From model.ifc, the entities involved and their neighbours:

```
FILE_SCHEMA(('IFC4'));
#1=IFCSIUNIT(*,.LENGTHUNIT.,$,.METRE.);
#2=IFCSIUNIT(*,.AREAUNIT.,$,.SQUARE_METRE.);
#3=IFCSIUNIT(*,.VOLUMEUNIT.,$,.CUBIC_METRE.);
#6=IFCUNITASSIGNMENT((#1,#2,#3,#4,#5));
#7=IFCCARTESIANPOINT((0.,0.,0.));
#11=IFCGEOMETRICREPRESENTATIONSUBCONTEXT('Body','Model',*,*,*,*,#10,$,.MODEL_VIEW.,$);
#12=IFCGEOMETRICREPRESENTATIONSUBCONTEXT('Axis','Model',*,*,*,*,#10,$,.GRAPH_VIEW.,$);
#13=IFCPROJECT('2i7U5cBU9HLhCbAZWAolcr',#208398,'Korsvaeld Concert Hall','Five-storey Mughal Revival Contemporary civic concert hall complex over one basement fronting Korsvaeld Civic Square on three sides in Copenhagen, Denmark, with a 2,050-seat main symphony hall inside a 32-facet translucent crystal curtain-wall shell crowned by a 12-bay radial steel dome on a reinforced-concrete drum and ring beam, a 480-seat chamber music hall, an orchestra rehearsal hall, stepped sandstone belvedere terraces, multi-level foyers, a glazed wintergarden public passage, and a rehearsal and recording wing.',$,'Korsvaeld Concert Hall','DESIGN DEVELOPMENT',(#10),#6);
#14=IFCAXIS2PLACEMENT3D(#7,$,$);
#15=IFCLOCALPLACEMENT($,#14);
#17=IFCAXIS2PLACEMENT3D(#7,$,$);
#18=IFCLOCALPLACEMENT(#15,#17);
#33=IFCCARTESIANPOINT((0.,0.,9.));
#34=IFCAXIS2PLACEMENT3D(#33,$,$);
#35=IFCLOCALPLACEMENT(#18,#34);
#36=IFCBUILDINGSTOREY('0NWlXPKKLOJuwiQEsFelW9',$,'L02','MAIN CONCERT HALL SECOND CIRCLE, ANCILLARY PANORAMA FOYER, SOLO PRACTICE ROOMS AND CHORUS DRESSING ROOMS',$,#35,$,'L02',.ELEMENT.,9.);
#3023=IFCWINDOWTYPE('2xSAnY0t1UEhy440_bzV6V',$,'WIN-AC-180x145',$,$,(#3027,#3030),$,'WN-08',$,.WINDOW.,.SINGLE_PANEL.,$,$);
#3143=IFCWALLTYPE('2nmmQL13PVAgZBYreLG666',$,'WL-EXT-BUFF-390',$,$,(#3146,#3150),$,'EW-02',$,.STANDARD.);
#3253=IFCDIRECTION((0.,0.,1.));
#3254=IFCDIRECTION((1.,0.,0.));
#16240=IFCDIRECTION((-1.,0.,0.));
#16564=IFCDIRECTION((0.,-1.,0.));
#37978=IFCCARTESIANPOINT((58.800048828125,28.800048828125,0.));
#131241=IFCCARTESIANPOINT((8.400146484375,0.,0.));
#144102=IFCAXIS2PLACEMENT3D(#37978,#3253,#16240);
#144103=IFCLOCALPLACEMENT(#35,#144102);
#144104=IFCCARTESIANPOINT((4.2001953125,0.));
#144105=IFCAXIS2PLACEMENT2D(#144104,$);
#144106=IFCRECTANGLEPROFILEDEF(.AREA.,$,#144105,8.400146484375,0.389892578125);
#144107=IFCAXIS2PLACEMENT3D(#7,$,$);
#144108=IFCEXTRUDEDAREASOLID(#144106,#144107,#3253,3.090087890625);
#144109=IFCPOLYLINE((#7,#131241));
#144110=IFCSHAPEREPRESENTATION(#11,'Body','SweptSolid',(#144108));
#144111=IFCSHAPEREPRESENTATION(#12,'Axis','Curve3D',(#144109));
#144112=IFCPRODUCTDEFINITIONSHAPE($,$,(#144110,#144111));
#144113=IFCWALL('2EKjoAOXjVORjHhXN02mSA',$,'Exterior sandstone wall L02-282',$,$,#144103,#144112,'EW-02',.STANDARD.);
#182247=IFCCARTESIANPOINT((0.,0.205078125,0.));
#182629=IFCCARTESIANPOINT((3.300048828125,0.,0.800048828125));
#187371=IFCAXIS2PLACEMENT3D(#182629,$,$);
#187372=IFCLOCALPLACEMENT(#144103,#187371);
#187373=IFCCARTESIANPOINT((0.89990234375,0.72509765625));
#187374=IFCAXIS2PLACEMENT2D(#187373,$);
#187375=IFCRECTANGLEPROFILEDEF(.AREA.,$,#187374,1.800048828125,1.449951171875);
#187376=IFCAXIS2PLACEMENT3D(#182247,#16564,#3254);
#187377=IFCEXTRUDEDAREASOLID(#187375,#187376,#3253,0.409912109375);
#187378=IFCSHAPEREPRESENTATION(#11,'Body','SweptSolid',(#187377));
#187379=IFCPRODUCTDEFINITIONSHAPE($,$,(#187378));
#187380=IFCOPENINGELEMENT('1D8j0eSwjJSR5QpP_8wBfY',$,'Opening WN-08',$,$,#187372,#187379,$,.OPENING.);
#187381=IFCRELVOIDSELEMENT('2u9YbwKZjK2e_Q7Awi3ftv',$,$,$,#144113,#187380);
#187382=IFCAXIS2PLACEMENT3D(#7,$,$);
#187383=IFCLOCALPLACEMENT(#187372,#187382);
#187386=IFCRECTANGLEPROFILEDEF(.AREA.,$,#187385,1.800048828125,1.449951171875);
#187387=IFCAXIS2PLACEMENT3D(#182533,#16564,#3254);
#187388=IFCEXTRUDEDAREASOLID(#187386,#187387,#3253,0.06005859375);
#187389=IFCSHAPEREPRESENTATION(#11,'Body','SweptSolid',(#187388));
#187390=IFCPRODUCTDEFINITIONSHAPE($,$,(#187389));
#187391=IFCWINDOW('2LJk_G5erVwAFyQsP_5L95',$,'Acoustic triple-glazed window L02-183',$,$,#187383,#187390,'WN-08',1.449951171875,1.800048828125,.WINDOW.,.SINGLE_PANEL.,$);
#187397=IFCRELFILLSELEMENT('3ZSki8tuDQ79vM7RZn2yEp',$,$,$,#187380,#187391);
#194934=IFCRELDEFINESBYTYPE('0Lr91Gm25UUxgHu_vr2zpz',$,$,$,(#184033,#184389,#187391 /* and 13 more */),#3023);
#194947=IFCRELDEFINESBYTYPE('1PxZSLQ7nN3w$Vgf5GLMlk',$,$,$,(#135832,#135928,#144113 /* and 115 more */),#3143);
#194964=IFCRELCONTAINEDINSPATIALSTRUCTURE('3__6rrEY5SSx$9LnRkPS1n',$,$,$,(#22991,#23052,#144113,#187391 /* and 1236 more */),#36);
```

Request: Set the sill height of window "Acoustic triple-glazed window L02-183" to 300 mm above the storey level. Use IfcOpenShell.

```python
import numpy as np
import ifcopenshell
import ifcopenshell.api.geometry
import ifcopenshell.geom
import ifcopenshell.util.element
import ifcopenshell.util.placement
import ifcopenshell.util.shape
import ifcopenshell.util.unit

model = ifcopenshell.open("model.ifc")
unit_scale = ifcopenshell.util.unit.calculate_unit_scale(model)

window = model.by_guid("2LJk_G5erVwAFyQsP_5L95")
opening = window.FillsVoids[0].RelatingOpeningElement
storey = ifcopenshell.util.element.get_container(window, ifc_class="IfcBuildingStorey")
level = ifcopenshell.util.placement.get_local_placement(storey.ObjectPlacement)[2, 3]

# The opening's origin need not be at the sill, so measure its lowest point.
shape = ifcopenshell.geom.create_shape(ifcopenshell.geom.settings(), opening)
bottom = ifcopenshell.util.shape.get_shape_bottom_elevation(shape, shape.geometry) / unit_scale
dz = level + 0.3 - bottom

shift = np.array([0.0, 0.0, dz])
# The window is placed relative to its opening, so it follows when the opening moves.
matrix = ifcopenshell.util.placement.get_local_placement(opening.ObjectPlacement)
matrix[:3, 3] += shift
ifcopenshell.api.geometry.edit_object_placement(
    model, product=opening, matrix=matrix, is_si=False, should_transform_children=True
)

print(f"moved by {dz * unit_scale:+.3f} m")

model.write("model_rev.ifc")
```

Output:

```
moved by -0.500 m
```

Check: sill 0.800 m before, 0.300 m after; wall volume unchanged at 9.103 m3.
